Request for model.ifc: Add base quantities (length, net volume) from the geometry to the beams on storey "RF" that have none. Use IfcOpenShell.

First a look at what the model holds.

```python
import ifcopenshell
import ifcopenshell.util.element
import ifcopenshell.util.unit

model = ifcopenshell.open("model.ifc")
print(model.schema)
for unit_type in ("LENGTHUNIT", "AREAUNIT", "VOLUMEUNIT"):
    print(unit_type, ifcopenshell.util.unit.calculate_unit_scale(model, unit_type))
storey = next(s for s in model.by_type("IfcBuildingStorey") if s.Name == "RF")
beams = [e for e in ifcopenshell.util.element.get_decomposition(storey) if e.is_a("IfcBeam")]
for e in sorted(beams, key=lambda e: e.id()):
    print(e.id(), e.is_a(), e.Name, list(ifcopenshell.util.element.get_psets(e, qtos_only=True)), sep=" | ")
```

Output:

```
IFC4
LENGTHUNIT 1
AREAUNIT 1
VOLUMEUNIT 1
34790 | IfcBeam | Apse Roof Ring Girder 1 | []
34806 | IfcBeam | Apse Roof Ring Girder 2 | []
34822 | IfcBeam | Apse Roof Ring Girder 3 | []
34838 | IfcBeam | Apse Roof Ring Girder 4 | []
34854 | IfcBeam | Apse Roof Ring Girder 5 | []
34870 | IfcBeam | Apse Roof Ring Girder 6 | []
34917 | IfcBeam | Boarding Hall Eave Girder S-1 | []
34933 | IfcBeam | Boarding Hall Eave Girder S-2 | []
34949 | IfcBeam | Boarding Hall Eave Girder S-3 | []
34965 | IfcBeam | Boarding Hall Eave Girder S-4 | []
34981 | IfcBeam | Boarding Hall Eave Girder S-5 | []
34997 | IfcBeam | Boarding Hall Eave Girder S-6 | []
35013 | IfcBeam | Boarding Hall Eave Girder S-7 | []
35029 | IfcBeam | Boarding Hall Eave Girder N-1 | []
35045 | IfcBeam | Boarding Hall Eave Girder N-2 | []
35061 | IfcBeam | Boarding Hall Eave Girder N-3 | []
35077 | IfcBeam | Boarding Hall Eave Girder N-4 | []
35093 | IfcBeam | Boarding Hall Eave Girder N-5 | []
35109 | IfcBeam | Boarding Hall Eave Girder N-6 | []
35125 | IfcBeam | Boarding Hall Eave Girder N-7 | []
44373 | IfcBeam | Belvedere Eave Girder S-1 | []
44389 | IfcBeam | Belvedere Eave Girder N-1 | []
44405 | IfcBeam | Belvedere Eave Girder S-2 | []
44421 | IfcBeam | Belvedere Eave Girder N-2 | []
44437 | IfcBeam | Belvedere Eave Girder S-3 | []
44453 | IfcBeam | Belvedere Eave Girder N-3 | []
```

```python
import ifcopenshell
import ifcopenshell.api.pset
import ifcopenshell.geom
import ifcopenshell.util.element
import ifcopenshell.util.shape
import ifcopenshell.util.unit

model = ifcopenshell.open("model.ifc")
unit_scale = ifcopenshell.util.unit.calculate_unit_scale(model)
volume_scale = ifcopenshell.util.unit.calculate_unit_scale(model, "VOLUMEUNIT")
settings = ifcopenshell.geom.settings()

storey = next(s for s in model.by_type("IfcBuildingStorey") if s.Name == "RF")
beams = [e for e in ifcopenshell.util.element.get_decomposition(storey) if e.is_a("IfcBeam")]

for e in sorted(beams, key=lambda e: e.id()):
    if ifcopenshell.util.element.get_psets(e, qtos_only=True, should_inherit=False):
        continue
    # Geometry comes back in metres, in the element's own axes.
    shape = ifcopenshell.geom.create_shape(settings, e)
    values = {
        "Length": ifcopenshell.util.shape.get_max_xyz(shape.geometry) / unit_scale,
        "NetVolume": ifcopenshell.util.shape.get_volume(shape.geometry) / volume_scale,
    }
    qto = ifcopenshell.api.pset.add_qto(model, product=e, name="Qto_BeamBaseQuantities")
    ifcopenshell.api.pset.edit_qto(model, qto=qto, properties=values)
    print(e.id(), {k: round(v, 3) for k, v in values.items()})

model.write("model_rev.ifc")
```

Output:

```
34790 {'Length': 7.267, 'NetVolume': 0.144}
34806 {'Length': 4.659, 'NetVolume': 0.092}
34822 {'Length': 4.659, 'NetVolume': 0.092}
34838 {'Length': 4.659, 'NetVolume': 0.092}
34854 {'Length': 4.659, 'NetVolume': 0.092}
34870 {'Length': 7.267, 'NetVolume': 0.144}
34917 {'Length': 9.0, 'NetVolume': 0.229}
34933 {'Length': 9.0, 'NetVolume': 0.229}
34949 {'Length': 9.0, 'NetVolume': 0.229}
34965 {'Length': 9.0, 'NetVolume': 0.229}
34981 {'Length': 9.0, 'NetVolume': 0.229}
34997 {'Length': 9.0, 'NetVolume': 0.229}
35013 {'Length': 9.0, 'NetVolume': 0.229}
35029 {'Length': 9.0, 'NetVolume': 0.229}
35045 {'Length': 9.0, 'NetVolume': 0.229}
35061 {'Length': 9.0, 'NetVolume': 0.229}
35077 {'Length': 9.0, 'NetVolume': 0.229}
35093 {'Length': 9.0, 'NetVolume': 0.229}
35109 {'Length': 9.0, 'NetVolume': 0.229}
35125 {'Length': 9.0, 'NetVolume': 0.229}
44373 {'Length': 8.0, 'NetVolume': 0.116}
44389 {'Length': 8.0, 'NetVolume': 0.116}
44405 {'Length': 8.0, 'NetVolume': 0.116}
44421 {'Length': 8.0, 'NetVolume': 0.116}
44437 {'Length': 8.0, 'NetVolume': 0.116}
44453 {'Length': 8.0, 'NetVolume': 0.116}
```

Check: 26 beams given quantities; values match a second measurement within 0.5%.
